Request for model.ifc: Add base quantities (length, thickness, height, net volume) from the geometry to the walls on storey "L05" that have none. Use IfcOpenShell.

First a look at what the model holds.

```python
import ifcopenshell
import ifcopenshell.util.element
import ifcopenshell.util.unit

model = ifcopenshell.open("model.ifc")
print(model.schema)
for unit_type in ("LENGTHUNIT", "AREAUNIT", "VOLUMEUNIT"):
    print(unit_type, ifcopenshell.util.unit.calculate_unit_scale(model, unit_type))
storey = next(s for s in model.by_type("IfcBuildingStorey") if s.Name == "L05")
walls = [e for e in ifcopenshell.util.element.get_decomposition(storey) if e.is_a("IfcWall")]
for e in sorted(walls, key=lambda e: e.id()):
    print(e.id(), e.is_a(), e.Name, list(ifcopenshell.util.element.get_psets(e, qtos_only=True)), sep=" | ")
```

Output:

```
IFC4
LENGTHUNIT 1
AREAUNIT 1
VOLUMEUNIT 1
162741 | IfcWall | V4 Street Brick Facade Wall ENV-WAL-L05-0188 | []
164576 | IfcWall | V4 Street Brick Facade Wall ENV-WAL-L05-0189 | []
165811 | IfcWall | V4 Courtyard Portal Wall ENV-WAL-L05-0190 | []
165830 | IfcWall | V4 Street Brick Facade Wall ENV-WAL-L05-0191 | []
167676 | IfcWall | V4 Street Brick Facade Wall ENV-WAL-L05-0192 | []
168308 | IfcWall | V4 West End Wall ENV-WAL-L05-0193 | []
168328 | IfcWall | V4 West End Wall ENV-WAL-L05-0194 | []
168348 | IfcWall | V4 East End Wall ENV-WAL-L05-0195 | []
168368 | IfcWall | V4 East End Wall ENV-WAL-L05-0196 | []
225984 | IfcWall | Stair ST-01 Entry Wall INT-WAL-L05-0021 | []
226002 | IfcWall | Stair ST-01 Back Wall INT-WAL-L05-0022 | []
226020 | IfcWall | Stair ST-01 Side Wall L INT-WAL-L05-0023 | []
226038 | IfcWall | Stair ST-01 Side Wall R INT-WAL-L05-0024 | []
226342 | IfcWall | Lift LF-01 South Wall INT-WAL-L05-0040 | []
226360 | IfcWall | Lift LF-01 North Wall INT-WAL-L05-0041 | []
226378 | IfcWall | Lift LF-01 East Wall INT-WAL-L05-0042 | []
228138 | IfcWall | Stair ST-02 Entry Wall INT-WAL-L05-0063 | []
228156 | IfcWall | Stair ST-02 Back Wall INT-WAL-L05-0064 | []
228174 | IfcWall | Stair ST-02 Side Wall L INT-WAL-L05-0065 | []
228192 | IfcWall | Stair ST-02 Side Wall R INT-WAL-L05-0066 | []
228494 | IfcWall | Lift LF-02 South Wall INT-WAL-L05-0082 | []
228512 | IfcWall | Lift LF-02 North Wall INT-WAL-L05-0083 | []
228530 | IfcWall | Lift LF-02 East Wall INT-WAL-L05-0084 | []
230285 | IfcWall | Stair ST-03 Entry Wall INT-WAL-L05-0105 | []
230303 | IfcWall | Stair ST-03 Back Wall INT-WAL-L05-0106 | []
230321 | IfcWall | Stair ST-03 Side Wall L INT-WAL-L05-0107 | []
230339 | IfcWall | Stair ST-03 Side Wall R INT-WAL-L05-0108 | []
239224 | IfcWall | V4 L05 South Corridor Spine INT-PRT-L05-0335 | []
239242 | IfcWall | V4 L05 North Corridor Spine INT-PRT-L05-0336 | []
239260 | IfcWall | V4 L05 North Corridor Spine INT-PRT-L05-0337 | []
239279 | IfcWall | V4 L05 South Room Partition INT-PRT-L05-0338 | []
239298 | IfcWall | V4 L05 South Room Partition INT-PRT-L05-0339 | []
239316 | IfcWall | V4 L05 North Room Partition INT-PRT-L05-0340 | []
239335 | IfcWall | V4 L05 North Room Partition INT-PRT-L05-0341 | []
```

```python
import ifcopenshell
import ifcopenshell.api.pset
import ifcopenshell.geom
import ifcopenshell.util.element
import ifcopenshell.util.shape
import ifcopenshell.util.unit

model = ifcopenshell.open("model.ifc")
unit_scale = ifcopenshell.util.unit.calculate_unit_scale(model)
volume_scale = ifcopenshell.util.unit.calculate_unit_scale(model, "VOLUMEUNIT")
settings = ifcopenshell.geom.settings()

storey = next(s for s in model.by_type("IfcBuildingStorey") if s.Name == "L05")
walls = [e for e in ifcopenshell.util.element.get_decomposition(storey) if e.is_a("IfcWall")]

for e in sorted(walls, key=lambda e: e.id()):
    if ifcopenshell.util.element.get_psets(e, qtos_only=True, should_inherit=False):
        continue
    # Geometry comes back in metres, in the element's own axes.
    shape = ifcopenshell.geom.create_shape(settings, e)
    values = {
        "Length": ifcopenshell.util.shape.get_x(shape.geometry) / unit_scale,
        "Width": ifcopenshell.util.shape.get_y(shape.geometry) / unit_scale,
        "Height": ifcopenshell.util.shape.get_z(shape.geometry) / unit_scale,
        "NetVolume": ifcopenshell.util.shape.get_volume(shape.geometry) / volume_scale,
    }
    qto = ifcopenshell.api.pset.add_qto(model, product=e, name="Qto_WallBaseQuantities")
    ifcopenshell.api.pset.edit_qto(model, qto=qto, properties=values)
    print(e.id(), {k: round(v, 3) for k, v in values.items()})

model.write("model_updated.ifc")
```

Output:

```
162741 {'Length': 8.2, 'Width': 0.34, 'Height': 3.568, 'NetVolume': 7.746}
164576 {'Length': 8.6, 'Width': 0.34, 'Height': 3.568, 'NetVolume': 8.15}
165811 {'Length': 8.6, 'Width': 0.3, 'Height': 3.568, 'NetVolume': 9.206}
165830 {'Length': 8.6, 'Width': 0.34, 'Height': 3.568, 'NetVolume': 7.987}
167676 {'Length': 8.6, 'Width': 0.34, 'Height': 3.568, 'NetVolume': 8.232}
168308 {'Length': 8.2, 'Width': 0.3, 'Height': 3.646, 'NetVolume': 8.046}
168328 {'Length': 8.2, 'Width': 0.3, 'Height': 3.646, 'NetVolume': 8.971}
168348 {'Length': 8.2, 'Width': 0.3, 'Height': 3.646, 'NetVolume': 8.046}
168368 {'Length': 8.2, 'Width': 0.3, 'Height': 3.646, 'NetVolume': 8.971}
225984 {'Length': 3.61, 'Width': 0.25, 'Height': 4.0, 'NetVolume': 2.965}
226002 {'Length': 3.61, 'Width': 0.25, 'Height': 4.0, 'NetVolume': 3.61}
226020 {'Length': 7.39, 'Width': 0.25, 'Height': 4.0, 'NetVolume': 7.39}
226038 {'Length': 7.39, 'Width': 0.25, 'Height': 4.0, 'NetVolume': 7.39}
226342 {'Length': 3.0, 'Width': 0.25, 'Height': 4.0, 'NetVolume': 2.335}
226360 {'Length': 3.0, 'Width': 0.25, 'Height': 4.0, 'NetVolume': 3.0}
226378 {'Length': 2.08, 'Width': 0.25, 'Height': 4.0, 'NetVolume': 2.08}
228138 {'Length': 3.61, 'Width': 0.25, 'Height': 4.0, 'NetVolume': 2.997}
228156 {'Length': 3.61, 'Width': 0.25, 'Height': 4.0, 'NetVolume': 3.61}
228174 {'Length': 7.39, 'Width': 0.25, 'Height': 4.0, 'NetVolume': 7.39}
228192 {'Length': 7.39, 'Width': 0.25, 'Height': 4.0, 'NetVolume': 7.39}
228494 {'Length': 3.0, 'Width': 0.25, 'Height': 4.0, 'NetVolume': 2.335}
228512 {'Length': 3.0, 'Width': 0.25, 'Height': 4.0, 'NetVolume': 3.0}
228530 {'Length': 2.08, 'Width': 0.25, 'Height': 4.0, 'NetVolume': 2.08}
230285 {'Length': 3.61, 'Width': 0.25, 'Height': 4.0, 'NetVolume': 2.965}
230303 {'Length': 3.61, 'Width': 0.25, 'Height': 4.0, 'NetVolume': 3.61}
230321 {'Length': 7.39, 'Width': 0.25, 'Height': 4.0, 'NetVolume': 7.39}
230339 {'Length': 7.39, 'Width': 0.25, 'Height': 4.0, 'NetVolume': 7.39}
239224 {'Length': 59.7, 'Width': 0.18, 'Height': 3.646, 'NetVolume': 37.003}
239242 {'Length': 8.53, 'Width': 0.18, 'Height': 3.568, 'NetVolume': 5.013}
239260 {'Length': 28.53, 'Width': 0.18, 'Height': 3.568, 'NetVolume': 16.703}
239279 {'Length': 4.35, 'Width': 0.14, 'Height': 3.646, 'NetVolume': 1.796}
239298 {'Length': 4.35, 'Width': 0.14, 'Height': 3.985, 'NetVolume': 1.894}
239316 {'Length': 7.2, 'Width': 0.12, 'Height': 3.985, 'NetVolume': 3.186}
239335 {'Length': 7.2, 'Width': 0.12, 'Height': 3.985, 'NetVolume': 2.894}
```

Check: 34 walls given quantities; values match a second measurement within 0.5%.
